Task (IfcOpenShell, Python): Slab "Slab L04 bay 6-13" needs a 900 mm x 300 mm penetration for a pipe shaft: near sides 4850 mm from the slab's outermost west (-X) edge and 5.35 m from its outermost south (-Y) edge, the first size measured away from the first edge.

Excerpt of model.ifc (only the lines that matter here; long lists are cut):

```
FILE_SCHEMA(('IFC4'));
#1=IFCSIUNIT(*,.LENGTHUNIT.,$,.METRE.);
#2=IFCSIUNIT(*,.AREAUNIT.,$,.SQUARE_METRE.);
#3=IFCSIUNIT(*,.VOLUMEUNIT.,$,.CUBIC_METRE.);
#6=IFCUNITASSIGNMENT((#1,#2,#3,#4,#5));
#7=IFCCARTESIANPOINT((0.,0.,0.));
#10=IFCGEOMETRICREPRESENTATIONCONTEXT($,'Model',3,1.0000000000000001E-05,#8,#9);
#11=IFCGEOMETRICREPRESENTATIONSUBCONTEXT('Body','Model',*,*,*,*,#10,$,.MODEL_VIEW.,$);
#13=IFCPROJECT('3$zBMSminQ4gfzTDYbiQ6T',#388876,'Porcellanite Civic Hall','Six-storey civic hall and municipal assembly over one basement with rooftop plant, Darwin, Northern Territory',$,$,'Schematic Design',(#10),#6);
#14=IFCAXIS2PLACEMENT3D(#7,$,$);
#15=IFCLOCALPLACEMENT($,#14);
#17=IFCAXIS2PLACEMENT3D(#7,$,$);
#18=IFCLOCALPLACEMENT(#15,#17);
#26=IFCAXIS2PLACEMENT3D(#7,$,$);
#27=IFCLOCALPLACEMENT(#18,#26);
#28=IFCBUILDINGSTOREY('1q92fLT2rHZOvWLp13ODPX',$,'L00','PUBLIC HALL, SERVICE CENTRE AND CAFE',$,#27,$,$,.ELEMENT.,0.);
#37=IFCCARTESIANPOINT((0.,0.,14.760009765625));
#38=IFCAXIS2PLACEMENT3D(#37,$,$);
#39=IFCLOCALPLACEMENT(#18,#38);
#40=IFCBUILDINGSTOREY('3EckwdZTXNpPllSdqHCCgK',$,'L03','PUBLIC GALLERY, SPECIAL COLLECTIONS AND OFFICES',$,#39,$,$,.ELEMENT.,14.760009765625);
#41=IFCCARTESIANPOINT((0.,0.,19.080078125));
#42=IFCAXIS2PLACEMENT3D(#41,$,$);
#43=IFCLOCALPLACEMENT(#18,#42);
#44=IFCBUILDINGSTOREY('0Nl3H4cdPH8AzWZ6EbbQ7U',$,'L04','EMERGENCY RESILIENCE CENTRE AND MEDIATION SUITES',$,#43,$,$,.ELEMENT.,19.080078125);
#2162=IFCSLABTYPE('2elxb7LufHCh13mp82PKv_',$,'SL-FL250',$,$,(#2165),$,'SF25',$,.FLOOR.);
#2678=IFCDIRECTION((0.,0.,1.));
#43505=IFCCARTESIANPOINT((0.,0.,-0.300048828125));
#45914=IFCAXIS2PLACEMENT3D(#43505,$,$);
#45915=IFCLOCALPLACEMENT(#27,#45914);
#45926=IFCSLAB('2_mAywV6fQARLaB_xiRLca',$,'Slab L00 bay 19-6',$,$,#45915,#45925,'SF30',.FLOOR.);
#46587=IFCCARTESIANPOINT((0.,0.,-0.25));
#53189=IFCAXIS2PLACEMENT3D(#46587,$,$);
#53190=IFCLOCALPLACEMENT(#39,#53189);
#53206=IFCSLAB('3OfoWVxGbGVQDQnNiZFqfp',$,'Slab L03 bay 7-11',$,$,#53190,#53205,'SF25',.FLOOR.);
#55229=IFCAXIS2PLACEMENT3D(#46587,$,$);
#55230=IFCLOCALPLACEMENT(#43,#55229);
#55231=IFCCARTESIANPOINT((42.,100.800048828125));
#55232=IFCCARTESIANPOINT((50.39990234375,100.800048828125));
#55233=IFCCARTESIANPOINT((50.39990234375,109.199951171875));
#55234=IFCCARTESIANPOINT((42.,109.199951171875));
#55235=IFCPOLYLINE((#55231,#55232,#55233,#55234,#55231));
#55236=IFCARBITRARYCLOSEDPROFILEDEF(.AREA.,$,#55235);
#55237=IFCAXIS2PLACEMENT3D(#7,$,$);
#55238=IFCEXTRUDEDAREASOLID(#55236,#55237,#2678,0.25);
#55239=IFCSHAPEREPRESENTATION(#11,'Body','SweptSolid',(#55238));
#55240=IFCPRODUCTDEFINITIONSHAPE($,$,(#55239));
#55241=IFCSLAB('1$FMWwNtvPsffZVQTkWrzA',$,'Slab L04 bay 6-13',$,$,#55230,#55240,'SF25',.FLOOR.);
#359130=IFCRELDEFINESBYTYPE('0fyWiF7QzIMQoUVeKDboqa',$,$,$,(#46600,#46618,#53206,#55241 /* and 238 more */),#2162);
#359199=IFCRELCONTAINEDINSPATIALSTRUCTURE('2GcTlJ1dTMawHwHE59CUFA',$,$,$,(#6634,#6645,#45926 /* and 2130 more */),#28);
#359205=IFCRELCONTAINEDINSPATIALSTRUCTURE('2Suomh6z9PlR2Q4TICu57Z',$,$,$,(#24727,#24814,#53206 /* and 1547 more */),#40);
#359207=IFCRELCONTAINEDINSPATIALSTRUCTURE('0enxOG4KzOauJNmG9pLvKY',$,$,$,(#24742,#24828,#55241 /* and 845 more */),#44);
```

```python
import numpy as np
import ifcopenshell
import ifcopenshell.api.feature
import ifcopenshell.api.geometry
import ifcopenshell.api.root
import ifcopenshell.geom
import ifcopenshell.util.placement
import ifcopenshell.util.representation
import ifcopenshell.util.shape
import ifcopenshell.util.unit

model = ifcopenshell.open("model.ifc")
unit_scale = ifcopenshell.util.unit.calculate_unit_scale(model)
settings = ifcopenshell.geom.settings()


def volume(element):
    """Net volume in cubic metres, openings subtracted."""
    shape = ifcopenshell.geom.create_shape(settings, element)
    return ifcopenshell.util.shape.get_volume(shape.geometry)


slab = model.by_id(55241)
before = volume(slab)

# Extent in the slab's own axes, in metres. The edges named are its -X and -Y sides.
slab_shape = ifcopenshell.geom.create_shape(settings, slab)
vertices = ifcopenshell.util.shape.get_vertices(slab_shape.geometry)
x_min, y_min, bottom = vertices.min(axis=0)
top = vertices[:, 2].max()

opening = ifcopenshell.api.root.create_entity(model, ifc_class="IfcOpeningElement", name="Pipe shaft opening", predefined_type="OPENING")
context = ifcopenshell.util.representation.get_context(model, "Model", "Body", "MODEL_VIEW")
width, depth = 0.9, 0.3
outline = [(0.0, 0.0), (width, 0.0), (width, depth), (0.0, depth), (0.0, 0.0)]
# Overshoot both faces by 50 mm so the cut is clean.
shape = ifcopenshell.api.geometry.add_slab_representation(
    model, context=context, depth=top - bottom + 0.1, polyline=outline
)
ifcopenshell.api.geometry.assign_representation(model, product=opening, representation=shape)

matrix = ifcopenshell.util.placement.get_local_placement(slab.ObjectPlacement)
matrix[:, 3] = matrix @ np.append(np.array([x_min + 4.85, y_min + 5.35, bottom - 0.05]) / unit_scale, 1.0)
ifcopenshell.api.geometry.edit_object_placement(model, product=opening, matrix=matrix, is_si=False)
ifcopenshell.api.feature.add_feature(model, feature=opening, element=slab)

after = volume(slab)

print(f"slab volume {before:.3f} -> {after:.3f} m3")

model.write("model_rev.ifc")
```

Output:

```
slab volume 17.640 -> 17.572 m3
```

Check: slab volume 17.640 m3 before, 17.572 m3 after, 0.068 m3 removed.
